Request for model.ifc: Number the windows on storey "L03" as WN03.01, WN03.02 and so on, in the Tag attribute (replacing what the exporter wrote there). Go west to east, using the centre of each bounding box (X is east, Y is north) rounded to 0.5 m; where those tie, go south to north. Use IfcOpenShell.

First a look at what the model holds.

```python
import ifcopenshell
import ifcopenshell.util.element
import ifcopenshell.util.placement

model = ifcopenshell.open("model.ifc")
print(model.schema)
storey = next(s for s in model.by_type("IfcBuildingStorey") if s.Name == "L03")
windows = [e for e in ifcopenshell.util.element.get_decomposition(storey) if e.is_a("IfcWindow")]
for e in sorted(windows, key=lambda e: e.id()):
    origin = ifcopenshell.util.placement.get_local_placement(e.ObjectPlacement)[:3, 3]
    print(e.id(), e.Tag, e.Name, origin.round(2) + 0.0, sep=" | ")
```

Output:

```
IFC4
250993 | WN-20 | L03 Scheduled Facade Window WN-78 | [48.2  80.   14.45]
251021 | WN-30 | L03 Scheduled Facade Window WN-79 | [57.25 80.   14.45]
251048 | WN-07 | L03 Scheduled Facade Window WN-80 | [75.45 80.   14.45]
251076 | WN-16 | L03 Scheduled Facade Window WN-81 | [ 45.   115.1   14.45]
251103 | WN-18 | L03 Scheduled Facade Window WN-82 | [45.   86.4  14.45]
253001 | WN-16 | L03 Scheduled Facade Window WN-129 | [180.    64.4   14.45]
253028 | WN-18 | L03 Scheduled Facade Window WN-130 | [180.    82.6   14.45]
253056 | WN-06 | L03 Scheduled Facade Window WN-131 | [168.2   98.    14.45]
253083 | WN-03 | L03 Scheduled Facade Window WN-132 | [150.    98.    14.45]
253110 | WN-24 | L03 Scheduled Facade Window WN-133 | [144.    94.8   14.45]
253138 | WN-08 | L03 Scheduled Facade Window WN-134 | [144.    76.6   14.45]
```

```python
import ifcopenshell
import ifcopenshell.geom
import ifcopenshell.util.element
import ifcopenshell.util.shape

model = ifcopenshell.open("model.ifc")
settings = ifcopenshell.geom.settings()
settings.set("use-world-coords", True)


def centre(element):
    shape = ifcopenshell.geom.create_shape(settings, element)
    return ifcopenshell.util.shape.get_bbox_centroid(shape.geometry)


storey = next(s for s in model.by_type("IfcBuildingStorey") if s.Name == "L03")
windows = [e for e in ifcopenshell.util.element.get_decomposition(storey) if e.is_a("IfcWindow")]

# Insertion points can sit at a corner or the storey origin, so sort by the geometry (in metres).
centres = {e: centre(e) for e in windows}
windows.sort(key=lambda e: (round(centres[e][0] / 0.5), centres[e][1]))

for i, e in enumerate(windows, start=1):
    number = f"WN03.{i:02d}"
    e.Tag = number
    print(e.id(), number)

model.write("model_edited.ifc")
```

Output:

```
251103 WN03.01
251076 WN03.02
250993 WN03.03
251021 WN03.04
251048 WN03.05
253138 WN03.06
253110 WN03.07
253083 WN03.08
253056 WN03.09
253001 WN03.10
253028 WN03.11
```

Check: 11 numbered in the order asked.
